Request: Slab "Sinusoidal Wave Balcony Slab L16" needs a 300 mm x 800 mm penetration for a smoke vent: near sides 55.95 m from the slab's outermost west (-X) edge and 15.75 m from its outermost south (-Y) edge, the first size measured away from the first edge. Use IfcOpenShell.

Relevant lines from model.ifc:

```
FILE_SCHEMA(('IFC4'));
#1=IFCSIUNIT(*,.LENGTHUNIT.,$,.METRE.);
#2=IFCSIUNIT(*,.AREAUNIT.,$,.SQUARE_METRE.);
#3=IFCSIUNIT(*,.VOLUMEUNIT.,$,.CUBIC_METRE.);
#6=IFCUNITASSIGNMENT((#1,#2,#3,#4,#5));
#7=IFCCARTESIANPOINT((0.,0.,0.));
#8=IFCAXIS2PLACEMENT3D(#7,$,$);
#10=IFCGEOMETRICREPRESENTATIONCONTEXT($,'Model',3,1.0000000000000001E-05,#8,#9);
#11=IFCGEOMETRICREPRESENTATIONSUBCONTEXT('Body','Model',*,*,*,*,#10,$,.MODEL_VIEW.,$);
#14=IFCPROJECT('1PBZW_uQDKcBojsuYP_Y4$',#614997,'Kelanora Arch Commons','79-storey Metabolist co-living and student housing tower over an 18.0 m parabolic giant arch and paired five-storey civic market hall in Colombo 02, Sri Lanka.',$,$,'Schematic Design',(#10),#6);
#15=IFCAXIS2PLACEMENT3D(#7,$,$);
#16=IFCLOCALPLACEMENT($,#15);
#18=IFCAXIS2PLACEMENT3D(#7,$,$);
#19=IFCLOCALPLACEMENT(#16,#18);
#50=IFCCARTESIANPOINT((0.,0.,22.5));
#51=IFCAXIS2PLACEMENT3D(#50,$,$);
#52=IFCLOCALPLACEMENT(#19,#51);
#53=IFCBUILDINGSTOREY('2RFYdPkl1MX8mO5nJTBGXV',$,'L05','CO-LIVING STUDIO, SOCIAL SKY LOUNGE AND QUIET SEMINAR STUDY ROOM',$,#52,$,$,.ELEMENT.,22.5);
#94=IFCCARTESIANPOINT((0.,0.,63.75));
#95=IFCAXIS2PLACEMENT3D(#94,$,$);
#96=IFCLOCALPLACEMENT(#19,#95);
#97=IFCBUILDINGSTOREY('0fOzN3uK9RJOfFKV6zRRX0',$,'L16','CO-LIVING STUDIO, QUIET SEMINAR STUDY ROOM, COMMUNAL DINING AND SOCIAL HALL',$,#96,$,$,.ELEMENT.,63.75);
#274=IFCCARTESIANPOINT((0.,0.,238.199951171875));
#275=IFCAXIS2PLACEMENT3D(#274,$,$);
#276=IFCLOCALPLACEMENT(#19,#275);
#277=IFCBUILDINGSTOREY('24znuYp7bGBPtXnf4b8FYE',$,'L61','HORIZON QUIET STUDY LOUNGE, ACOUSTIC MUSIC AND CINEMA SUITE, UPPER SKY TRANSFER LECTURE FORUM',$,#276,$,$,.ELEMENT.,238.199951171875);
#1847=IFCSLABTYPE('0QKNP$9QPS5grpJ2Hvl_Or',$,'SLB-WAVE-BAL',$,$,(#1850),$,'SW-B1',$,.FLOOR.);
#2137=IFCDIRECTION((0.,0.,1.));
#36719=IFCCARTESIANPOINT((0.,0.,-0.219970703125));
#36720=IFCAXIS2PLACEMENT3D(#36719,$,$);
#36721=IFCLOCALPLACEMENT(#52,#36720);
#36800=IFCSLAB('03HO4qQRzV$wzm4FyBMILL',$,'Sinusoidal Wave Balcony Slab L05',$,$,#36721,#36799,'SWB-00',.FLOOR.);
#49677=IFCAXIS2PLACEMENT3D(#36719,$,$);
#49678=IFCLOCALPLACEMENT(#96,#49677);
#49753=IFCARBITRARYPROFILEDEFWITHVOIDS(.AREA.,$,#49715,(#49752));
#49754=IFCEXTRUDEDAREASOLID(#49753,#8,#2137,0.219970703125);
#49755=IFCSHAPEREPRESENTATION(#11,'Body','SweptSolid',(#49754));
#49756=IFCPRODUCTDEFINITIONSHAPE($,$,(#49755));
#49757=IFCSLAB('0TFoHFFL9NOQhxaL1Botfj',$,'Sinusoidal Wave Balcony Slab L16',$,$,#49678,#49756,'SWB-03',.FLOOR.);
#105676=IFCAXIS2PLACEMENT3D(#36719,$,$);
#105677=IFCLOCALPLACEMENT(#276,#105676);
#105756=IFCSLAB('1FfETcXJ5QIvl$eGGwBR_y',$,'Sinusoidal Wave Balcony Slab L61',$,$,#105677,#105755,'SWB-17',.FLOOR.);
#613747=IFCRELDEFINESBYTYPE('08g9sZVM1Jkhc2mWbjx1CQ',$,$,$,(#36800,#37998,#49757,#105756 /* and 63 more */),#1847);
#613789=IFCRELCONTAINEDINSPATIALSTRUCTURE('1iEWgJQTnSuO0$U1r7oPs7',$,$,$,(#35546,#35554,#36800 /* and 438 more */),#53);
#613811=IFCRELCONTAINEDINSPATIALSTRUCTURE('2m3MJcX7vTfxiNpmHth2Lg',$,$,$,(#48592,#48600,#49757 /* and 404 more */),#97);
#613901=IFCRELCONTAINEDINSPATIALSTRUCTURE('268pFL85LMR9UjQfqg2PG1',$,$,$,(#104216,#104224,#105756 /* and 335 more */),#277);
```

```python
import numpy as np
import ifcopenshell
import ifcopenshell.api.feature
import ifcopenshell.api.geometry
import ifcopenshell.api.root
import ifcopenshell.geom
import ifcopenshell.util.placement
import ifcopenshell.util.representation
import ifcopenshell.util.shape
import ifcopenshell.util.unit

model = ifcopenshell.open("model.ifc")
unit_scale = ifcopenshell.util.unit.calculate_unit_scale(model)
settings = ifcopenshell.geom.settings()


def volume(element):
    """Net volume in cubic metres, openings subtracted."""
    shape = ifcopenshell.geom.create_shape(settings, element)
    return ifcopenshell.util.shape.get_volume(shape.geometry)


slab = model.by_id(49757)
before = volume(slab)

# Extent in the slab's own axes, in metres. The edges named are its -X and -Y sides.
slab_shape = ifcopenshell.geom.create_shape(settings, slab)
vertices = ifcopenshell.util.shape.get_vertices(slab_shape.geometry)
x_min, y_min, bottom = vertices.min(axis=0)
top = vertices[:, 2].max()

opening = ifcopenshell.api.root.create_entity(model, ifc_class="IfcOpeningElement", name="Smoke vent opening", predefined_type="OPENING")
context = ifcopenshell.util.representation.get_context(model, "Model", "Body", "MODEL_VIEW")
width, depth = 0.3, 0.8
outline = [(0.0, 0.0), (width, 0.0), (width, depth), (0.0, depth), (0.0, 0.0)]
# Overshoot both faces by 50 mm so the cut is clean.
shape = ifcopenshell.api.geometry.add_slab_representation(
    model, context=context, depth=top - bottom + 0.1, polyline=outline
)
ifcopenshell.api.geometry.assign_representation(model, product=opening, representation=shape)

matrix = ifcopenshell.util.placement.get_local_placement(slab.ObjectPlacement)
matrix[:, 3] = matrix @ np.append(np.array([x_min + 55.95, y_min + 15.75, bottom - 0.05]) / unit_scale, 1.0)
ifcopenshell.api.geometry.edit_object_placement(model, product=opening, matrix=matrix, is_si=False)
ifcopenshell.api.feature.add_feature(model, feature=opening, element=slab)

after = volume(slab)

print(f"slab volume {before:.3f} -> {after:.3f} m3")

model.write("model_edited.ifc")
```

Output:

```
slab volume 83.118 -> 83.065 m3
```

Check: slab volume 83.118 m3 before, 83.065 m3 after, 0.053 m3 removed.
